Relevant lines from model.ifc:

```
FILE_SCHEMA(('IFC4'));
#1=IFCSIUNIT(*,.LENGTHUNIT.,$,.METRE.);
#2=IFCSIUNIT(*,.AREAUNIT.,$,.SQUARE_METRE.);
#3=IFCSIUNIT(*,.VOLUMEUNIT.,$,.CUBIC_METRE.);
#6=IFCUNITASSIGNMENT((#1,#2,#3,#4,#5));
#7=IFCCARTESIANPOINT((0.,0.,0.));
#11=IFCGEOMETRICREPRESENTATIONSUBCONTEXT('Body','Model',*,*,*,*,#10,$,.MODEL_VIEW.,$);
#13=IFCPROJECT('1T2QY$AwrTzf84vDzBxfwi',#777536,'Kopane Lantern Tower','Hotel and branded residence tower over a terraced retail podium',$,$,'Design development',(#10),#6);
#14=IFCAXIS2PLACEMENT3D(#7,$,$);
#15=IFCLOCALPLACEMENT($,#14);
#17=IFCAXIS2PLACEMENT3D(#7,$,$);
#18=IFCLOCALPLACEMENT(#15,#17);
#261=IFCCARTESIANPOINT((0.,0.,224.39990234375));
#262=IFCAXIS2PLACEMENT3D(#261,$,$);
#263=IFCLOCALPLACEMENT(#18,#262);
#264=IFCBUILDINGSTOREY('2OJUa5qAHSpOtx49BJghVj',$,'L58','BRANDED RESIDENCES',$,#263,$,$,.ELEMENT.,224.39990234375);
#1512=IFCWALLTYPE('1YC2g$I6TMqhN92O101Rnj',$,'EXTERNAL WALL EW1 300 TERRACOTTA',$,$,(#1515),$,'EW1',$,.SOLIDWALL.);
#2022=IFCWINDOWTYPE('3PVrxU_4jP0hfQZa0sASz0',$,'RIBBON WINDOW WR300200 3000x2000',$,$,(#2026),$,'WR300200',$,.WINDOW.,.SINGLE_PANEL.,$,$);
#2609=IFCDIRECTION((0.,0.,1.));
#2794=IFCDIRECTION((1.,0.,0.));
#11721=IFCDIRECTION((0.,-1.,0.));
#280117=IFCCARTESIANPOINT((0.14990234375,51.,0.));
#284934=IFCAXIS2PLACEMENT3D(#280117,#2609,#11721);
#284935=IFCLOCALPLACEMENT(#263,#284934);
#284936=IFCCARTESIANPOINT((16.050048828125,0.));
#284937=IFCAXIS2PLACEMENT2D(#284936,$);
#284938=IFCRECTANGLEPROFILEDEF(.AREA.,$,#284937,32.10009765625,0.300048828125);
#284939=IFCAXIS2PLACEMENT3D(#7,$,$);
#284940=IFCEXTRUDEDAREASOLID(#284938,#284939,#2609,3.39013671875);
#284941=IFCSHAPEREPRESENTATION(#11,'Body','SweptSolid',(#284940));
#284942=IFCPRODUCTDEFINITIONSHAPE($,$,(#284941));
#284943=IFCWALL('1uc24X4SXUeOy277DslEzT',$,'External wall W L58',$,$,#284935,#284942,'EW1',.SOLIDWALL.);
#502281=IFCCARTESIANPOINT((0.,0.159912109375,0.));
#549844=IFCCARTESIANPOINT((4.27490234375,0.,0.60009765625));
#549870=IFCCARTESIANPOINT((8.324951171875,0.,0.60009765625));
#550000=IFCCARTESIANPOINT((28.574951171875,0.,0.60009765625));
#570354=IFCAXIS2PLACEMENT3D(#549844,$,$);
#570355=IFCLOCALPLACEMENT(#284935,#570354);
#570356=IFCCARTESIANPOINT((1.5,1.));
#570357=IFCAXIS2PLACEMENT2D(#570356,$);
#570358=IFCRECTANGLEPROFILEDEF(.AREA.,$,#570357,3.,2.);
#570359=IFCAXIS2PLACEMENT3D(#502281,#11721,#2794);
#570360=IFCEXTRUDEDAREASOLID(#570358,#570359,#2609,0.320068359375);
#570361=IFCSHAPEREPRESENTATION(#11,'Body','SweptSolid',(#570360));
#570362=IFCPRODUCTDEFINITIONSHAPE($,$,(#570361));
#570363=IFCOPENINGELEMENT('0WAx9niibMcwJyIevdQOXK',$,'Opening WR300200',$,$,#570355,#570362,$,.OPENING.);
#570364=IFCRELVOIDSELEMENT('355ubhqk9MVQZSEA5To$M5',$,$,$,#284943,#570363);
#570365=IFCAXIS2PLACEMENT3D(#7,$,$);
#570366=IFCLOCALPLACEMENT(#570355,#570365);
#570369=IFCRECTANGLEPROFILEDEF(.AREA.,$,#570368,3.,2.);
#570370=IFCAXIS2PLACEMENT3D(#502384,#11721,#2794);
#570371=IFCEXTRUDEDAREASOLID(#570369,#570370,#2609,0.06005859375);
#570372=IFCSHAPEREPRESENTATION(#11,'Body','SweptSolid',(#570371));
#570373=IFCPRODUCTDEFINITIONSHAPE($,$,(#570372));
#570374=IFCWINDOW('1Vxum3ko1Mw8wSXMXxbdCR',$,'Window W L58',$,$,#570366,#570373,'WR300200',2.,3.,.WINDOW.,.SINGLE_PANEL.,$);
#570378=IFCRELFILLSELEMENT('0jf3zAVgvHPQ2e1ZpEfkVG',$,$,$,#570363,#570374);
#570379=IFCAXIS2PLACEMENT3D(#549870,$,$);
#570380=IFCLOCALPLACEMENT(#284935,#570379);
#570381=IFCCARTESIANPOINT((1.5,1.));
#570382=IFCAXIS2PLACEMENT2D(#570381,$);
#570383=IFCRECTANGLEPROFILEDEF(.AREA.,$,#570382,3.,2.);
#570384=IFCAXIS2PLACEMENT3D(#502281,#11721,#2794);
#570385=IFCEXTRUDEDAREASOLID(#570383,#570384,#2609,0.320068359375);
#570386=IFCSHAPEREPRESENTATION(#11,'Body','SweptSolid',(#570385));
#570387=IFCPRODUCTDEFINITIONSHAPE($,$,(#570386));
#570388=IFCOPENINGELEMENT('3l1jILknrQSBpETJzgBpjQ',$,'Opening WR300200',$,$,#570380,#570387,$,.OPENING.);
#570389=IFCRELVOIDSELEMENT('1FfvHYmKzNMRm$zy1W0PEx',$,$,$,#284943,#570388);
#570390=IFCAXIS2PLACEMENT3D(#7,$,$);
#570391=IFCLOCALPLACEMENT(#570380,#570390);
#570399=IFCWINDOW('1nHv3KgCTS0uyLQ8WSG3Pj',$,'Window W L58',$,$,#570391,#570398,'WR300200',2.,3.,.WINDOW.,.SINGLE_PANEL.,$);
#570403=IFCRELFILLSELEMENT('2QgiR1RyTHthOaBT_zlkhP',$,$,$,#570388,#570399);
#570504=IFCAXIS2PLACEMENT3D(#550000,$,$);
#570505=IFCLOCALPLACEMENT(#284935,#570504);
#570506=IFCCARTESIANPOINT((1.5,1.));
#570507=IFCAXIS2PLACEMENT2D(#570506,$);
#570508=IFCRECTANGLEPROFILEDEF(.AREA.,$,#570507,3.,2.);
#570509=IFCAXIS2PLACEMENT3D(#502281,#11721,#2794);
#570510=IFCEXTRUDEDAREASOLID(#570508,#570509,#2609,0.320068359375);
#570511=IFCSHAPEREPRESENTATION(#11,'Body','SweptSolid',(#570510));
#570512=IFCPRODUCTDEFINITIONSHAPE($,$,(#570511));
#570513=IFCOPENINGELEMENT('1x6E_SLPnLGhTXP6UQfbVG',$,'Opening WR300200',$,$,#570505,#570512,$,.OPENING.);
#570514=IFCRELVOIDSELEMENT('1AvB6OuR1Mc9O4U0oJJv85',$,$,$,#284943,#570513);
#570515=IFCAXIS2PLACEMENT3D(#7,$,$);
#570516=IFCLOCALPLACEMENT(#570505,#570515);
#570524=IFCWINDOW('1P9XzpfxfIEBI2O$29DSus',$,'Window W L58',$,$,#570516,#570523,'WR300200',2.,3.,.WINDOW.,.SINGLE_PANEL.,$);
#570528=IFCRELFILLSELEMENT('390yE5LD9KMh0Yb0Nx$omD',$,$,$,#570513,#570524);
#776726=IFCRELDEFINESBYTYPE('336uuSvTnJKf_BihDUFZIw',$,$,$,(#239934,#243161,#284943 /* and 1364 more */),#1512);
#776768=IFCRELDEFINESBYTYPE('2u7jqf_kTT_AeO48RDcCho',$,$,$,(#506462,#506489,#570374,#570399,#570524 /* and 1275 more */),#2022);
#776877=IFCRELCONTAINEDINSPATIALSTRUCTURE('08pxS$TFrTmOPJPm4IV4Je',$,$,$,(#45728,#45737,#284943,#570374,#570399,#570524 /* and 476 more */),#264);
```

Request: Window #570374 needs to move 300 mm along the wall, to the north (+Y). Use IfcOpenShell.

```python
import ifcopenshell
import ifcopenshell.api.geometry
import ifcopenshell.util.placement
import ifcopenshell.util.unit

model = ifcopenshell.open("model.ifc")
unit_scale = ifcopenshell.util.unit.calculate_unit_scale(model)

window = model.by_guid("1Vxum3ko1Mw8wSXMXxbdCR")
opening = window.FillsVoids[0].RelatingOpeningElement
wall = opening.VoidsElements[0].RelatingBuildingElement

wall_matrix = ifcopenshell.util.placement.get_local_placement(wall.ObjectPlacement)
shift = wall_matrix[:3, 0] * -0.3 / unit_scale
before = ifcopenshell.util.placement.get_local_placement(window.ObjectPlacement)[:3, 3].copy()

# The window is placed relative to its opening, so it follows when the opening moves.
matrix = ifcopenshell.util.placement.get_local_placement(opening.ObjectPlacement)
matrix[:3, 3] += shift
ifcopenshell.api.geometry.edit_object_placement(
    model, product=opening, matrix=matrix, is_si=False, should_transform_children=True
)

after = ifcopenshell.util.placement.get_local_placement(window.ObjectPlacement)[:3, 3]
print("window moved by", (after - before).round(3) + 0.0)

model.write("model_v2.ifc")
```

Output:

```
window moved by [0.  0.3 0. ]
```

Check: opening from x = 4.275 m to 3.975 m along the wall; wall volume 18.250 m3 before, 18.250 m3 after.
